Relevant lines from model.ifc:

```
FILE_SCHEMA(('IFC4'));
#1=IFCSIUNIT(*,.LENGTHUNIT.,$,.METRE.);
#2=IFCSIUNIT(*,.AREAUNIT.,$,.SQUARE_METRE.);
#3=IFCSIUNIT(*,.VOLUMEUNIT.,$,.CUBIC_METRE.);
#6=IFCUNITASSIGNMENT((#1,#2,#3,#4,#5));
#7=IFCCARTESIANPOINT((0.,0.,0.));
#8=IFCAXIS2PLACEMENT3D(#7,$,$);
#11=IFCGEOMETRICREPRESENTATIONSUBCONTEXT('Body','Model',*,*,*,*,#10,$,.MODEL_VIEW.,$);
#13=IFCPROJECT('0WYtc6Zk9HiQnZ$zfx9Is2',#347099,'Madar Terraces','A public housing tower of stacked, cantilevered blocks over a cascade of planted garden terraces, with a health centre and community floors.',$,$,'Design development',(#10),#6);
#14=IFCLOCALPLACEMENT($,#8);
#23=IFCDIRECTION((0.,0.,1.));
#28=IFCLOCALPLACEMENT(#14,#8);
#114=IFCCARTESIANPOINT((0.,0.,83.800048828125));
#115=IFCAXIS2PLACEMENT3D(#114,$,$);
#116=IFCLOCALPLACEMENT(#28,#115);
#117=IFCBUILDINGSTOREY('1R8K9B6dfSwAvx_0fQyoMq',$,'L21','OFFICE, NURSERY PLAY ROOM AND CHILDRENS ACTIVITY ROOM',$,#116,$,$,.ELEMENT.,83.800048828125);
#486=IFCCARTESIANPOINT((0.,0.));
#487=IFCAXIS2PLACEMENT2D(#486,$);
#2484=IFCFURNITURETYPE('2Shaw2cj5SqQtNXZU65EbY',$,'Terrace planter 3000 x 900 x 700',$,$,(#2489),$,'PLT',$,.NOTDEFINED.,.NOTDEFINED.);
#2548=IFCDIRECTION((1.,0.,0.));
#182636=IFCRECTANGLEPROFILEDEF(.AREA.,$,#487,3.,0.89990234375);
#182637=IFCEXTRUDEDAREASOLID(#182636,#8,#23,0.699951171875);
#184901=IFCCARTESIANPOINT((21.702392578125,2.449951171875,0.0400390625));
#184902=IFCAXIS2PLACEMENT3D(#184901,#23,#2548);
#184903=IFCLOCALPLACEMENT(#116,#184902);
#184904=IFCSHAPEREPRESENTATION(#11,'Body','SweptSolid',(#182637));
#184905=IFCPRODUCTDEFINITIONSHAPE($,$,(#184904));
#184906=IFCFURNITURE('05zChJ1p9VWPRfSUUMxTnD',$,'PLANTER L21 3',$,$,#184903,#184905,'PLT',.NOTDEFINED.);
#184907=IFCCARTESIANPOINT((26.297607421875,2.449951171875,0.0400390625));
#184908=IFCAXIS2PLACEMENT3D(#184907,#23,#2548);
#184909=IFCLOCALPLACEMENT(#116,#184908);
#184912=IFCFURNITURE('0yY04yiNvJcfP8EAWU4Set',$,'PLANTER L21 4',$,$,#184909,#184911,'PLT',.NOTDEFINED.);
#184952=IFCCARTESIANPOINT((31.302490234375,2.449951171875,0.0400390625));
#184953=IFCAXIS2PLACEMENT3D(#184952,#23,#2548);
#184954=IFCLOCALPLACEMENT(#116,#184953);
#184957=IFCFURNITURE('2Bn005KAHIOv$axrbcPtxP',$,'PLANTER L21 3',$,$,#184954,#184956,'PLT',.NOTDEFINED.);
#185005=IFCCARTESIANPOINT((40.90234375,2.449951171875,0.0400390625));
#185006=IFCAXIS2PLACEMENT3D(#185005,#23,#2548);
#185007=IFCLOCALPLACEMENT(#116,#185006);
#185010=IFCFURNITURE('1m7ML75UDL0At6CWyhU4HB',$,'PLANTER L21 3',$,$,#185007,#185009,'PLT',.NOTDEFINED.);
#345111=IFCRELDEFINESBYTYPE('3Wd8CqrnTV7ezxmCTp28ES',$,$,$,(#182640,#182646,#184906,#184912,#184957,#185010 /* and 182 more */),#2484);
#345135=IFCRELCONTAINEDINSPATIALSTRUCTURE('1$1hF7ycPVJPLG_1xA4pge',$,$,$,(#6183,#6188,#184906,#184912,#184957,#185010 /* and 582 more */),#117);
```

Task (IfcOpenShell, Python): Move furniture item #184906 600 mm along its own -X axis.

```python
import ifcopenshell
import ifcopenshell.api.geometry
import ifcopenshell.util.placement
import ifcopenshell.util.unit

model = ifcopenshell.open("model.ifc")
unit_scale = ifcopenshell.util.unit.calculate_unit_scale(model)

item = model.by_guid("05zChJ1p9VWPRfSUUMxTnD")
matrix = ifcopenshell.util.placement.get_local_placement(item.ObjectPlacement)
matrix[:3, 3] -= matrix[:3, 0] * 0.6 / unit_scale
ifcopenshell.api.geometry.edit_object_placement(model, product=item, matrix=matrix, is_si=False)

print(ifcopenshell.util.placement.get_local_placement(item.ObjectPlacement).round(3) + 0.0)

model.write("model-out.ifc")
```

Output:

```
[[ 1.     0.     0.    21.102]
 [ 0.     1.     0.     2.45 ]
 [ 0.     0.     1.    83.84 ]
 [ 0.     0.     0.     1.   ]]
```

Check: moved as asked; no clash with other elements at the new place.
